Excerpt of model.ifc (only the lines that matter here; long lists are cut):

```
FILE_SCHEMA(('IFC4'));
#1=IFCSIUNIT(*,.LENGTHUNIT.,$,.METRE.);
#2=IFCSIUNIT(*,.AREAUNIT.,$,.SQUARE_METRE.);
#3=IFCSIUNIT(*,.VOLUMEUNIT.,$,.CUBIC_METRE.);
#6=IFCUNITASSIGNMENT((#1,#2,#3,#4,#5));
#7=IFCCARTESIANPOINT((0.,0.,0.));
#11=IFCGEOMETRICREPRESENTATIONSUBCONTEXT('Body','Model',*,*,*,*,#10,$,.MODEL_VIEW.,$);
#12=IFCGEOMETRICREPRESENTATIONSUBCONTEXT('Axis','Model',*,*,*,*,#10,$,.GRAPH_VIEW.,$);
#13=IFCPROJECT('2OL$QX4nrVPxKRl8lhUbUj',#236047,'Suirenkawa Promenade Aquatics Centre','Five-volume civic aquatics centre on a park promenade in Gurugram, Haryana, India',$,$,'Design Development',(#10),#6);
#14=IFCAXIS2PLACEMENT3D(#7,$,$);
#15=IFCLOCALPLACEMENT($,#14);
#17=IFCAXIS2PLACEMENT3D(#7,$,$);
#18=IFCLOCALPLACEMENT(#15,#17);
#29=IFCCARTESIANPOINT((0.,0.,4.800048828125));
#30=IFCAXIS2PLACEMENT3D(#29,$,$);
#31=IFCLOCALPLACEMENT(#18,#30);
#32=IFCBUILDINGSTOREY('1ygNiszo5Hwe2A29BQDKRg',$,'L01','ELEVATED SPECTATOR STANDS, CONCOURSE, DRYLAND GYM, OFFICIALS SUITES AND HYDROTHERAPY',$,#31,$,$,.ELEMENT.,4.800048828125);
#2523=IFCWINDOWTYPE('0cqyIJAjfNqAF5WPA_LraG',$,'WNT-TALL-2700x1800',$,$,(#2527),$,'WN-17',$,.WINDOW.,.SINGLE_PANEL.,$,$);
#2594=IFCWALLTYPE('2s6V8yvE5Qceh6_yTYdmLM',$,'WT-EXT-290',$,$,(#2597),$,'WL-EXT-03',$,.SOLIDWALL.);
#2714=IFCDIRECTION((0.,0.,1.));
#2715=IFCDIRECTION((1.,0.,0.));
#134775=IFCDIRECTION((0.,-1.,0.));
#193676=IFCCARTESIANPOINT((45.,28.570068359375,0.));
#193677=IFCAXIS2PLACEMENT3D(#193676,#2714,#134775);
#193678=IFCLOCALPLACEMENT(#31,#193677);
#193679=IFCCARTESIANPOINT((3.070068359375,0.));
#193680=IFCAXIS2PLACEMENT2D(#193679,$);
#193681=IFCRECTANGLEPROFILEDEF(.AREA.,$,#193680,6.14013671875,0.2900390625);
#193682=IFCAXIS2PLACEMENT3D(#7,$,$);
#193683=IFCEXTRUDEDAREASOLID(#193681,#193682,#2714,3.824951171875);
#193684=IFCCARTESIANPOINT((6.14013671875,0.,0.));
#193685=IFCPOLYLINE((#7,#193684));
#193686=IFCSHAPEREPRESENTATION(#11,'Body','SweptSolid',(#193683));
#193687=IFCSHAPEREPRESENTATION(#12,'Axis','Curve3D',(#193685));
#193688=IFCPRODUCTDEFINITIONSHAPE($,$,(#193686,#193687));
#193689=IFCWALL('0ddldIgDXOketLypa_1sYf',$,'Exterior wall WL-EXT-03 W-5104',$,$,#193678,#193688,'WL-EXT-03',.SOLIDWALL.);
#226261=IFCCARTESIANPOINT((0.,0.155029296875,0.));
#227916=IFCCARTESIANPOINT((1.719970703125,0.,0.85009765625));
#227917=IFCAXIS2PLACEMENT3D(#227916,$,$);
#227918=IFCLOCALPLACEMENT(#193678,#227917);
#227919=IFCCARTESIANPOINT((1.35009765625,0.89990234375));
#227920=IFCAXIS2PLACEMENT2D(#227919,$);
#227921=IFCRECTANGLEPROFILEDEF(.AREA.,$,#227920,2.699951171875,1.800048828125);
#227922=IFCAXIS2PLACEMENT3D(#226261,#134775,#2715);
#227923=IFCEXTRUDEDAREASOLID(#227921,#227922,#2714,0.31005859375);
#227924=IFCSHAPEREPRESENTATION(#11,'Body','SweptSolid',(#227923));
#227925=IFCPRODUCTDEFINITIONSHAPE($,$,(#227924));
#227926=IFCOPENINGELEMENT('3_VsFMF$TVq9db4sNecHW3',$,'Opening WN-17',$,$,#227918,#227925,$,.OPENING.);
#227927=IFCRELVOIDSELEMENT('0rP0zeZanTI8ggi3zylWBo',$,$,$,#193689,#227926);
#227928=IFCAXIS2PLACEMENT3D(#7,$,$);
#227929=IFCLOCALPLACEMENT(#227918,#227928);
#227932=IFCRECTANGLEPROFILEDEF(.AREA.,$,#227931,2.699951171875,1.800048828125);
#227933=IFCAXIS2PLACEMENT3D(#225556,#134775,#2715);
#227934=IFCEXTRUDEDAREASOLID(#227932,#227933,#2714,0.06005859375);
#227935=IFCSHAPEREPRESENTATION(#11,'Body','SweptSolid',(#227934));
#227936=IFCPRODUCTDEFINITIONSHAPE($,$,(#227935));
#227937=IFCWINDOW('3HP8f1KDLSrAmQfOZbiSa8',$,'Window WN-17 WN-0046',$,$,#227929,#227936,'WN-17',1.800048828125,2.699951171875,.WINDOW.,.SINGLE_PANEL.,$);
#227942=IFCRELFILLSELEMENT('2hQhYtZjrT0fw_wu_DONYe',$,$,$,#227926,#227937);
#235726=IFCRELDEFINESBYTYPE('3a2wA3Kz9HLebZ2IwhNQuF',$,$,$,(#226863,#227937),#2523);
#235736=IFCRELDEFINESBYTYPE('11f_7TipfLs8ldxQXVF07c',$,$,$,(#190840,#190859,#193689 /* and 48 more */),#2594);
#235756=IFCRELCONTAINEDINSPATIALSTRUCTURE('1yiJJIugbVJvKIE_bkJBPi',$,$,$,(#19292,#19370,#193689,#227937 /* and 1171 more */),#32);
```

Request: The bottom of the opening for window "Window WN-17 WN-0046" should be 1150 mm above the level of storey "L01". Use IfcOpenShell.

```python
import numpy as np
import ifcopenshell
import ifcopenshell.api.geometry
import ifcopenshell.geom
import ifcopenshell.util.element
import ifcopenshell.util.placement
import ifcopenshell.util.shape
import ifcopenshell.util.unit

model = ifcopenshell.open("model.ifc")
unit_scale = ifcopenshell.util.unit.calculate_unit_scale(model)

window = model.by_guid("3HP8f1KDLSrAmQfOZbiSa8")
opening = window.FillsVoids[0].RelatingOpeningElement
storey = ifcopenshell.util.element.get_container(window, ifc_class="IfcBuildingStorey")
level = ifcopenshell.util.placement.get_local_placement(storey.ObjectPlacement)[2, 3]

# The opening's origin need not be at the sill, so measure its lowest point.
shape = ifcopenshell.geom.create_shape(ifcopenshell.geom.settings(), opening)
bottom = ifcopenshell.util.shape.get_shape_bottom_elevation(shape, shape.geometry) / unit_scale
dz = level + 1.15 / unit_scale - bottom

shift = np.array([0.0, 0.0, dz])
# The window is placed relative to its opening, so it follows when the opening moves.
matrix = ifcopenshell.util.placement.get_local_placement(opening.ObjectPlacement)
matrix[:3, 3] += shift
ifcopenshell.api.geometry.edit_object_placement(
    model, product=opening, matrix=matrix, is_si=False, should_transform_children=True
)

print(f"moved by {dz * unit_scale:+.3f} m")

model.write("model_rev.ifc")
```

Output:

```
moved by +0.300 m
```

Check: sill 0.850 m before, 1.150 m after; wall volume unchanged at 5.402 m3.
